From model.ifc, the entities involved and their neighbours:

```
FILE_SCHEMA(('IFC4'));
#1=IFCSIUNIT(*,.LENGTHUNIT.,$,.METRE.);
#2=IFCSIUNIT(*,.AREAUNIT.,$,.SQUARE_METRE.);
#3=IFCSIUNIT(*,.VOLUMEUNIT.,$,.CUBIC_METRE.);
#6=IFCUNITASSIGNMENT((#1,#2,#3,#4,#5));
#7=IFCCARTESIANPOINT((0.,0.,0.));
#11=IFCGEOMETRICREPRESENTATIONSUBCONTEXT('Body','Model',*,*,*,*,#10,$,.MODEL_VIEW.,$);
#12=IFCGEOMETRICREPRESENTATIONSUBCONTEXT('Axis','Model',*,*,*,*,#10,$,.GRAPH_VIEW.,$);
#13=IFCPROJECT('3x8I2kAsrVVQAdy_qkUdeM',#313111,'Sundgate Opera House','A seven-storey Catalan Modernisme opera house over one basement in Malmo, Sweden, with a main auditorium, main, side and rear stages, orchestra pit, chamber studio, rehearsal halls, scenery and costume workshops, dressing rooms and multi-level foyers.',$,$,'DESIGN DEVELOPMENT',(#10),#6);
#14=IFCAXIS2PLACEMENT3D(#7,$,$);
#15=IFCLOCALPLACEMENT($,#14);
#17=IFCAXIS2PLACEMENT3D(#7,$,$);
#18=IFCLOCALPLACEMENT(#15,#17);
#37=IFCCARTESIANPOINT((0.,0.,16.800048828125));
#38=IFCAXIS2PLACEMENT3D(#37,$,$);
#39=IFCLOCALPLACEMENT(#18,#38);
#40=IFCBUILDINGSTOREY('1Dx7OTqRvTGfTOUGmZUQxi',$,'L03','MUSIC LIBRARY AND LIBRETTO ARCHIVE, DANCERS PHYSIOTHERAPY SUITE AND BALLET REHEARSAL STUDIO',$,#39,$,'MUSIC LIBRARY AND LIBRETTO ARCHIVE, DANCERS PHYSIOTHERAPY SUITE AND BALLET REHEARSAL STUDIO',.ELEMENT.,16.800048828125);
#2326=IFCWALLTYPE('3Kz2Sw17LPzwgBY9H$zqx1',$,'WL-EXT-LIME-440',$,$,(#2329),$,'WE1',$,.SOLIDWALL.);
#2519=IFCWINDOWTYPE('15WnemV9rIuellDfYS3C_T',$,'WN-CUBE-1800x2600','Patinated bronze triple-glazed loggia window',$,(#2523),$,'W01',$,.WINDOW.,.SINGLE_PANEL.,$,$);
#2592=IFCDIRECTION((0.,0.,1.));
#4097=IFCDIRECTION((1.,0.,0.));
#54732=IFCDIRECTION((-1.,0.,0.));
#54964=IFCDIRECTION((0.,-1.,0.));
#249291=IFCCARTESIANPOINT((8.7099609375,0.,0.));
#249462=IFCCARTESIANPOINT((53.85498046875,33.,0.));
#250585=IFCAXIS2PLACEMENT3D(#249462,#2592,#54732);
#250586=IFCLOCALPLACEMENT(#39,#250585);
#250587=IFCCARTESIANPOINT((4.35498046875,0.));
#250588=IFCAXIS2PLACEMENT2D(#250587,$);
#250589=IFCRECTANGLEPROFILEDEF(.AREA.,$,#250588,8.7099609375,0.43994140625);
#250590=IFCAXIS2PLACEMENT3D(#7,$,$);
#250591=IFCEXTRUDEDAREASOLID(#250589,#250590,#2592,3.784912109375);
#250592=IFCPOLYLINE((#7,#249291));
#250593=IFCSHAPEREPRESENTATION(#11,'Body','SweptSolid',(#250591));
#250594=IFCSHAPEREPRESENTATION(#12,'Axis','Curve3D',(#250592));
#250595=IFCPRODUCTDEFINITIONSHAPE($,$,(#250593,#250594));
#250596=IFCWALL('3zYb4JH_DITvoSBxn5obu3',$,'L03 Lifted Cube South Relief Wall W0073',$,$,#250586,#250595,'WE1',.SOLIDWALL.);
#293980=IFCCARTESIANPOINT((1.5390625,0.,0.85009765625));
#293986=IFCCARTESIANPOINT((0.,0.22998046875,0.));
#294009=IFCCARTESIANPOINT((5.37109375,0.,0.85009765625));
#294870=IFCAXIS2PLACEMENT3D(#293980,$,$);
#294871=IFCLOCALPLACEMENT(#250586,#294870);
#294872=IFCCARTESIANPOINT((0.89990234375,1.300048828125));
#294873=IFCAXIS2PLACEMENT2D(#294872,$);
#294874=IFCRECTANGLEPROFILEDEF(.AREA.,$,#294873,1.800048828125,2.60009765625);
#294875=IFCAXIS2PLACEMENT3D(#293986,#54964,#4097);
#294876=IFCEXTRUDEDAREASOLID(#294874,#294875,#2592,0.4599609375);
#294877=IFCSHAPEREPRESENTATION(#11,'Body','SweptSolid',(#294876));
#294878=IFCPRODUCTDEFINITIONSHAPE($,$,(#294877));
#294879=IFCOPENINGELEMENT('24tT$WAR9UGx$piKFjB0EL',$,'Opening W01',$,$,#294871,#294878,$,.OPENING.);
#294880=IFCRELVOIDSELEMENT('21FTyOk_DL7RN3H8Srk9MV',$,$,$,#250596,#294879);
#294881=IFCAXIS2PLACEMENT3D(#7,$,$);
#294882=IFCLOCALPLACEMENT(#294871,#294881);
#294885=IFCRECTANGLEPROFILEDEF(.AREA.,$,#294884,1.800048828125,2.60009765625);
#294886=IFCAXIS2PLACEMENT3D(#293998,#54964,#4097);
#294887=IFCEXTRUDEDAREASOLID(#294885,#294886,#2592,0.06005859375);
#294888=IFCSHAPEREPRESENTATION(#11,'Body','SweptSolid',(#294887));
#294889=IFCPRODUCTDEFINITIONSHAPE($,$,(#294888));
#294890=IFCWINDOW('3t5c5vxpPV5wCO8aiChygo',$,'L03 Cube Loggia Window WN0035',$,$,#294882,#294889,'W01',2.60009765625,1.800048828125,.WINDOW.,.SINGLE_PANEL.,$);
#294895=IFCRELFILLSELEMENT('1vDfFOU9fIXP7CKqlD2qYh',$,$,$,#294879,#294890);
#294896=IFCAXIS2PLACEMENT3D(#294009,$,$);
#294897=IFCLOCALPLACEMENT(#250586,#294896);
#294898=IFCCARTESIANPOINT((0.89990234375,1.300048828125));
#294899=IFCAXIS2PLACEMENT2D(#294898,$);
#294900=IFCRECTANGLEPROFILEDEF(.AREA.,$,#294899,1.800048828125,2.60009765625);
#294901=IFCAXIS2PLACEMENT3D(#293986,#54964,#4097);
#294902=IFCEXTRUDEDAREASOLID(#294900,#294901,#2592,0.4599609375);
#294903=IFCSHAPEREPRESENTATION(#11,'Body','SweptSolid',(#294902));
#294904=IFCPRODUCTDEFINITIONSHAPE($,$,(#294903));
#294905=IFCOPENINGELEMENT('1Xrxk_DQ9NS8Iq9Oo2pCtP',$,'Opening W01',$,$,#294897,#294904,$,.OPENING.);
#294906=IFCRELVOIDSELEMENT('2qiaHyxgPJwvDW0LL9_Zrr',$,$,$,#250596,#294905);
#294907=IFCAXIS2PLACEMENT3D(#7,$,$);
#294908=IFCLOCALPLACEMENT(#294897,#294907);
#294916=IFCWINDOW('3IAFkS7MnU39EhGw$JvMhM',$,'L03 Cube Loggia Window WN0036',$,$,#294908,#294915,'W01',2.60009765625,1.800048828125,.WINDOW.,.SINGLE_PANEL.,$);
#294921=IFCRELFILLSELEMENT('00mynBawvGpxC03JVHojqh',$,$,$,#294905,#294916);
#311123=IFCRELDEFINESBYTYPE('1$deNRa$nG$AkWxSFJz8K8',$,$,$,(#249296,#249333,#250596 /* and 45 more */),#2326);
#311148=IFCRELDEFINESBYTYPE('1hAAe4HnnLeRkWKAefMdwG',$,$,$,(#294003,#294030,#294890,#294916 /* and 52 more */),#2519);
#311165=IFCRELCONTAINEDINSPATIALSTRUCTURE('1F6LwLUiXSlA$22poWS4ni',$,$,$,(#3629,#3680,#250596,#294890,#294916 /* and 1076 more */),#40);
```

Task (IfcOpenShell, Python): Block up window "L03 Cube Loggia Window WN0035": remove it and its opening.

```python
import ifcopenshell
import ifcopenshell.api.feature
import ifcopenshell.api.root
import ifcopenshell.geom
import ifcopenshell.util.shape

model = ifcopenshell.open("model.ifc")
settings = ifcopenshell.geom.settings()


def volume(element):
    """Net volume in cubic metres, openings subtracted."""
    shape = ifcopenshell.geom.create_shape(settings, element)
    return ifcopenshell.util.shape.get_volume(shape.geometry)


window = model.by_guid("3t5c5vxpPV5wCO8aiChygo")
opening = window.FillsVoids[0].RelatingOpeningElement
wall = opening.VoidsElements[0].RelatingBuildingElement
before = volume(wall)

ifcopenshell.api.root.remove_product(model, product=window)
ifcopenshell.api.feature.remove_feature(model, feature=opening)

after = volume(wall)

print(f"wall volume {before:.3f} -> {after:.3f} m3")

model.write("model_updated.ifc")
```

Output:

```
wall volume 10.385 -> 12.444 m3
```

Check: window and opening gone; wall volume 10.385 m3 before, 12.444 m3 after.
